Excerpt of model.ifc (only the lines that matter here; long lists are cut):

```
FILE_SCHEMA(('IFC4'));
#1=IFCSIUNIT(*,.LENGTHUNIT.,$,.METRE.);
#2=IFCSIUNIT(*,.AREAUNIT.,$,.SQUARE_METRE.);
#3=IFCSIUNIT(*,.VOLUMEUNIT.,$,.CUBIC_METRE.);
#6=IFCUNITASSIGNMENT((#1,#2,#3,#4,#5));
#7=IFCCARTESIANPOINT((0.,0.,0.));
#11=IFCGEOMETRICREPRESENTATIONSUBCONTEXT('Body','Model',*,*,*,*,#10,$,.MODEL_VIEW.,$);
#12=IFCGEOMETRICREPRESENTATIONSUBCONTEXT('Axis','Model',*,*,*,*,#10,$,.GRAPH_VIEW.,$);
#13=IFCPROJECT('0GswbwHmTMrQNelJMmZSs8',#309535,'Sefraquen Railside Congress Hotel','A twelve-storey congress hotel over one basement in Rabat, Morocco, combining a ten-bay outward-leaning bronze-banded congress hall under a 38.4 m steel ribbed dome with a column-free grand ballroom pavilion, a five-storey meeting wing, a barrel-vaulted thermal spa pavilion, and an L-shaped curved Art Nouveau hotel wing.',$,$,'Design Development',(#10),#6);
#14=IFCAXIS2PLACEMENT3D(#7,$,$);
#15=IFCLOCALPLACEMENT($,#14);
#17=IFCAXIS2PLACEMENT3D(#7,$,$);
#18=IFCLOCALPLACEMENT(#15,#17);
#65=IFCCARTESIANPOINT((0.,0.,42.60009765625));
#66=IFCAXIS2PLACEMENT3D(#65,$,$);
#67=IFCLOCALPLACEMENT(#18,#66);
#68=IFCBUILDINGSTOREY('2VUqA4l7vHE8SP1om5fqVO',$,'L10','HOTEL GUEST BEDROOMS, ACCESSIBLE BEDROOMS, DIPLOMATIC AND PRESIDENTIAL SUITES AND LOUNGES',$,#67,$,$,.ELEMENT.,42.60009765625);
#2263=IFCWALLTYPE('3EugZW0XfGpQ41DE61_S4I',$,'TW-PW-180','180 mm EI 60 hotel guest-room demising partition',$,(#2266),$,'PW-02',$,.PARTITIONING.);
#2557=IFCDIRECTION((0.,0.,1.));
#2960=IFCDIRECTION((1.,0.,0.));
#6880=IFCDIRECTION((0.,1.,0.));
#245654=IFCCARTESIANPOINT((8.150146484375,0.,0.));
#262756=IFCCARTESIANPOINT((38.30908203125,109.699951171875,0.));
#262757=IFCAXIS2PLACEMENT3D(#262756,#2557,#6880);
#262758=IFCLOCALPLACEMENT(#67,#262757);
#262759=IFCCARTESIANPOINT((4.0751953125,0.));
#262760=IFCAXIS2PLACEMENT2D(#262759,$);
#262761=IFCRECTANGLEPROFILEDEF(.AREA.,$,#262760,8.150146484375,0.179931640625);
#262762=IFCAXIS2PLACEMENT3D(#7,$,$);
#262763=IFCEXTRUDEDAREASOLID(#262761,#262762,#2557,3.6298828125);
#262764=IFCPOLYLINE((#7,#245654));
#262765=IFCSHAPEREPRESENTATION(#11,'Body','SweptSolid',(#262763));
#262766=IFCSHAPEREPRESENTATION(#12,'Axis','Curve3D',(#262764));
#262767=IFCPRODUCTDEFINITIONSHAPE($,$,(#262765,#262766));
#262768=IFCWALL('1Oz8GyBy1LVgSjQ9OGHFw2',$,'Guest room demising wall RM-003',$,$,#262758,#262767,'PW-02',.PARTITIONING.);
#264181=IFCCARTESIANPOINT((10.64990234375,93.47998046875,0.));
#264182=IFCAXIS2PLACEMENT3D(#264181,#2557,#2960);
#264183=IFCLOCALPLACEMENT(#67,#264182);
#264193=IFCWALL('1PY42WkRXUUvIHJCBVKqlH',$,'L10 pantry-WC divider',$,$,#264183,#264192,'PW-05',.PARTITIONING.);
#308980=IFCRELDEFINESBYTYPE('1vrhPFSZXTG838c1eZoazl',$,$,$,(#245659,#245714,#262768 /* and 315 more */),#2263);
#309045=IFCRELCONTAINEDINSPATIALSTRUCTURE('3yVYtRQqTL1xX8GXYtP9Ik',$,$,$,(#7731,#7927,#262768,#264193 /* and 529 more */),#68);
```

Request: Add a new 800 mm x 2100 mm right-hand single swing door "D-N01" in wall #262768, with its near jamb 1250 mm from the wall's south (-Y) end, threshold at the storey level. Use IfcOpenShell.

```python
import numpy as np
import ifcopenshell
import ifcopenshell.api.feature
import ifcopenshell.api.geometry
import ifcopenshell.api.root
import ifcopenshell.api.spatial
import ifcopenshell.geom
import ifcopenshell.util.element
import ifcopenshell.util.placement
import ifcopenshell.util.representation
import ifcopenshell.util.shape
import ifcopenshell.util.unit

model = ifcopenshell.open("model.ifc")
unit_scale = ifcopenshell.util.unit.calculate_unit_scale(model)
settings = ifcopenshell.geom.settings()


def volume(element):
    """Net volume in cubic metres, openings subtracted."""
    shape = ifcopenshell.geom.create_shape(settings, element)
    return ifcopenshell.util.shape.get_volume(shape.geometry)


wall = model.by_guid("1Oz8GyBy1LVgSjQ9OGHFw2")
storey = ifcopenshell.util.element.get_container(wall, ifc_class="IfcBuildingStorey")
context = ifcopenshell.util.representation.get_context(model, "Model", "Body", "MODEL_VIEW")
before = volume(wall)

width, height, from_end, sill = 0.8, 2.1, 1.25, 0.0  # metres

# The wall runs along its own X axis, and the end named is its -X end.
wall_shape = ifcopenshell.geom.create_shape(settings, wall)
x, y, z = ifcopenshell.util.shape.get_vertices(wall_shape.geometry).T
start = x.min() + from_end
face, thickness = float(y.min()), float(y.max() - y.min())
wall_matrix = ifcopenshell.util.placement.get_local_placement(wall.ObjectPlacement)
level = ifcopenshell.util.placement.get_local_placement(storey.ObjectPlacement)[2, 3]


def in_wall(x, y):
    """Placement at x, y metres in the wall's axes, at sill height."""
    matrix = wall_matrix.copy()
    matrix[:, 3] = wall_matrix @ np.array([x / unit_scale, y / unit_scale, 0.0, 1.0])
    matrix[2, 3] = level + sill / unit_scale
    return matrix


# Opening: a box that overshoots both wall faces by 50 mm.
opening = ifcopenshell.api.root.create_entity(model, ifc_class="IfcOpeningElement", predefined_type="OPENING")
box = ifcopenshell.api.geometry.add_wall_representation(
    model, context=context, length=width, height=height, thickness=thickness + 0.1
)
ifcopenshell.api.geometry.assign_representation(model, product=opening, representation=box)
ifcopenshell.api.geometry.edit_object_placement(model, product=opening, matrix=in_wall(start, face - 0.05), is_si=False)
ifcopenshell.api.feature.add_feature(model, feature=opening, element=wall)

door = ifcopenshell.api.root.create_entity(model, ifc_class="IfcDoor", name="D-N01", predefined_type="DOOR")
door.OverallWidth, door.OverallHeight = width / unit_scale, height / unit_scale
door.OperationType = "SINGLE_SWING_RIGHT"
body = ifcopenshell.api.geometry.add_door_representation(
    model,
    context=context,
    overall_width=door.OverallWidth,
    overall_height=door.OverallHeight,
    operation_type="SINGLE_SWING_RIGHT",
    lining_properties={"LiningDepth": thickness / unit_scale, "ThresholdDepth": thickness / unit_scale},
)
ifcopenshell.api.geometry.assign_representation(model, product=door, representation=body)
ifcopenshell.api.spatial.assign_container(model, products=[door], relating_structure=storey)
ifcopenshell.api.feature.add_filling(model, opening=opening, element=door)

# The lining spans the wall, so the door starts at the wall face.
ifcopenshell.api.geometry.edit_object_placement(model, product=door, matrix=in_wall(start, face), is_si=False)

after = volume(wall)

print(f"wall volume {before:.3f} -> {after:.3f} m3")

model.write("model_edited.ifc")
```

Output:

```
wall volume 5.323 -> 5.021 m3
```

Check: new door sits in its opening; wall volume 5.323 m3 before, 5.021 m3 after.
